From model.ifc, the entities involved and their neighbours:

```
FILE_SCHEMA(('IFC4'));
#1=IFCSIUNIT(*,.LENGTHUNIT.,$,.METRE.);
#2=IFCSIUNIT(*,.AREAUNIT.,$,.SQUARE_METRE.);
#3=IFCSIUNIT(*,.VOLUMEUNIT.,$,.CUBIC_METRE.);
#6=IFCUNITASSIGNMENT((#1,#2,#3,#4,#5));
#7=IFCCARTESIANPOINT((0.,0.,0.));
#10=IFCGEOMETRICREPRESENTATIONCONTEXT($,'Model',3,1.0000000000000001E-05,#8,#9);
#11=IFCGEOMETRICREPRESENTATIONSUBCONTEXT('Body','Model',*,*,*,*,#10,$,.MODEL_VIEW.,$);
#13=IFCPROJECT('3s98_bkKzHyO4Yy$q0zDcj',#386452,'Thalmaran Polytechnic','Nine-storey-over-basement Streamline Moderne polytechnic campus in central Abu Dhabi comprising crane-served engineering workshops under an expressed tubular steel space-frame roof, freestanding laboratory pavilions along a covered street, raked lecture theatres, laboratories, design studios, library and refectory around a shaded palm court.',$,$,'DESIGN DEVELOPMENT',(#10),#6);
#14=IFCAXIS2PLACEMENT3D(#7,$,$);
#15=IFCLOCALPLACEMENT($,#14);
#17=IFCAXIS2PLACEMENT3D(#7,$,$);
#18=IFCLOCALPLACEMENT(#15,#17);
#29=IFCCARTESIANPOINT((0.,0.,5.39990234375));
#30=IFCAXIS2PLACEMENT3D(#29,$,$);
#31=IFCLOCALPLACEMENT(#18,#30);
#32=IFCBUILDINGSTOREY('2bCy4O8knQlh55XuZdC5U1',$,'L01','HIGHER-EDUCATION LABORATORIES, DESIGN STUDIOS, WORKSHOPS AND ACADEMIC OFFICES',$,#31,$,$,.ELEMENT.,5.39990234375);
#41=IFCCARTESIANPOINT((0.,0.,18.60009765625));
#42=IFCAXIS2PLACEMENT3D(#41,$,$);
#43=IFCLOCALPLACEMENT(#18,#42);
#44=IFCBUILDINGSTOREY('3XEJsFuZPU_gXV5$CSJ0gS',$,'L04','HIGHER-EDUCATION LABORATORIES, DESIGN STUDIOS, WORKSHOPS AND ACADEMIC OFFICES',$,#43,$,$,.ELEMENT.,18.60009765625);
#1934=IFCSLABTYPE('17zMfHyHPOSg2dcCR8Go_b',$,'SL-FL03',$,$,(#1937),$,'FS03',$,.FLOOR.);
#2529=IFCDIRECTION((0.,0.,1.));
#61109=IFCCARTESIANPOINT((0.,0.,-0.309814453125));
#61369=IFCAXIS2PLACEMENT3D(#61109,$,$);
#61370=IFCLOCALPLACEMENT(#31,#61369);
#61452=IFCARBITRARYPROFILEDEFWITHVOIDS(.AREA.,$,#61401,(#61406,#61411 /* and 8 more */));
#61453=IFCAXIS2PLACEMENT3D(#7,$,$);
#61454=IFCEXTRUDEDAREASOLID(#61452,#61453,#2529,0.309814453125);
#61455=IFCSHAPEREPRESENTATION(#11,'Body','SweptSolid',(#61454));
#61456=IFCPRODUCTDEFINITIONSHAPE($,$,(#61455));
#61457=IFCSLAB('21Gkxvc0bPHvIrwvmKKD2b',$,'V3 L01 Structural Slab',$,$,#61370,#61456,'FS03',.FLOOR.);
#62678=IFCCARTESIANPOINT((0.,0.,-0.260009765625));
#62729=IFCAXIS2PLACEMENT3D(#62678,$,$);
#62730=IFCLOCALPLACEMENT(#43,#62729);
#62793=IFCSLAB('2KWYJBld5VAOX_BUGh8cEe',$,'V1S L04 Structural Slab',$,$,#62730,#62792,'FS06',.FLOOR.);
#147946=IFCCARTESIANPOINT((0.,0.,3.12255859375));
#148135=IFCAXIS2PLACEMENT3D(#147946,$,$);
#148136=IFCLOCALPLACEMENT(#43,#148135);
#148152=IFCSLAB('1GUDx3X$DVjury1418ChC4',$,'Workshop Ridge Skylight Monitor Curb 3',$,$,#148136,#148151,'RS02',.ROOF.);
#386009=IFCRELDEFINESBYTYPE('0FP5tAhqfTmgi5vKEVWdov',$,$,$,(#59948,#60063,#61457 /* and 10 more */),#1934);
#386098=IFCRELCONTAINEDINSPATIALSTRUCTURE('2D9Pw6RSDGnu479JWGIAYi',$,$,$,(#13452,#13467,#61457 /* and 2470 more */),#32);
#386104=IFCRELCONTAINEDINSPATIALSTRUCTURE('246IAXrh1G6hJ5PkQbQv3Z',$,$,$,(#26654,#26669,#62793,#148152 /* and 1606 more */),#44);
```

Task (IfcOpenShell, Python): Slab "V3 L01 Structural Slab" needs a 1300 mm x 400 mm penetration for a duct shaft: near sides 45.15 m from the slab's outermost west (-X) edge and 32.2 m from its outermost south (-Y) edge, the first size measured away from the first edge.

```python
import numpy as np
import ifcopenshell
import ifcopenshell.api.feature
import ifcopenshell.api.geometry
import ifcopenshell.api.root
import ifcopenshell.geom
import ifcopenshell.util.placement
import ifcopenshell.util.representation
import ifcopenshell.util.shape
import ifcopenshell.util.unit

model = ifcopenshell.open("model.ifc")
unit_scale = ifcopenshell.util.unit.calculate_unit_scale(model)
settings = ifcopenshell.geom.settings()


def volume(element):
    """Net volume in cubic metres, openings subtracted."""
    shape = ifcopenshell.geom.create_shape(settings, element)
    return ifcopenshell.util.shape.get_volume(shape.geometry)


slab = model.by_guid("21Gkxvc0bPHvIrwvmKKD2b")
before = volume(slab)

# Extent in the slab's own axes, in metres. The edges named are its -X and -Y sides.
slab_shape = ifcopenshell.geom.create_shape(settings, slab)
vertices = ifcopenshell.util.shape.get_vertices(slab_shape.geometry)
x_min, y_min, bottom = vertices.min(axis=0)
top = vertices[:, 2].max()

opening = ifcopenshell.api.root.create_entity(model, ifc_class="IfcOpeningElement", name="Duct shaft opening", predefined_type="OPENING")
context = ifcopenshell.util.representation.get_context(model, "Model", "Body", "MODEL_VIEW")
width, depth = 1.3, 0.4
outline = [(0.0, 0.0), (width, 0.0), (width, depth), (0.0, depth), (0.0, 0.0)]
# Overshoot both faces by 50 mm so the cut is clean.
shape = ifcopenshell.api.geometry.add_slab_representation(
    model, context=context, depth=top - bottom + 0.1, polyline=outline
)
ifcopenshell.api.geometry.assign_representation(model, product=opening, representation=shape)

matrix = ifcopenshell.util.placement.get_local_placement(slab.ObjectPlacement)
matrix[:, 3] = matrix @ np.append(np.array([x_min + 45.15, y_min + 32.2, bottom - 0.05]) / unit_scale, 1.0)
ifcopenshell.api.geometry.edit_object_placement(model, product=opening, matrix=matrix, is_si=False)
ifcopenshell.api.feature.add_feature(model, feature=opening, element=slab)

after = volume(slab)

print(f"slab volume {before:.3f} -> {after:.3f} m3")

model.write("model_rev.ifc")
```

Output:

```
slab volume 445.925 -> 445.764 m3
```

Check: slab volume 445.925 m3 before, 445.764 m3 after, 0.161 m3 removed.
